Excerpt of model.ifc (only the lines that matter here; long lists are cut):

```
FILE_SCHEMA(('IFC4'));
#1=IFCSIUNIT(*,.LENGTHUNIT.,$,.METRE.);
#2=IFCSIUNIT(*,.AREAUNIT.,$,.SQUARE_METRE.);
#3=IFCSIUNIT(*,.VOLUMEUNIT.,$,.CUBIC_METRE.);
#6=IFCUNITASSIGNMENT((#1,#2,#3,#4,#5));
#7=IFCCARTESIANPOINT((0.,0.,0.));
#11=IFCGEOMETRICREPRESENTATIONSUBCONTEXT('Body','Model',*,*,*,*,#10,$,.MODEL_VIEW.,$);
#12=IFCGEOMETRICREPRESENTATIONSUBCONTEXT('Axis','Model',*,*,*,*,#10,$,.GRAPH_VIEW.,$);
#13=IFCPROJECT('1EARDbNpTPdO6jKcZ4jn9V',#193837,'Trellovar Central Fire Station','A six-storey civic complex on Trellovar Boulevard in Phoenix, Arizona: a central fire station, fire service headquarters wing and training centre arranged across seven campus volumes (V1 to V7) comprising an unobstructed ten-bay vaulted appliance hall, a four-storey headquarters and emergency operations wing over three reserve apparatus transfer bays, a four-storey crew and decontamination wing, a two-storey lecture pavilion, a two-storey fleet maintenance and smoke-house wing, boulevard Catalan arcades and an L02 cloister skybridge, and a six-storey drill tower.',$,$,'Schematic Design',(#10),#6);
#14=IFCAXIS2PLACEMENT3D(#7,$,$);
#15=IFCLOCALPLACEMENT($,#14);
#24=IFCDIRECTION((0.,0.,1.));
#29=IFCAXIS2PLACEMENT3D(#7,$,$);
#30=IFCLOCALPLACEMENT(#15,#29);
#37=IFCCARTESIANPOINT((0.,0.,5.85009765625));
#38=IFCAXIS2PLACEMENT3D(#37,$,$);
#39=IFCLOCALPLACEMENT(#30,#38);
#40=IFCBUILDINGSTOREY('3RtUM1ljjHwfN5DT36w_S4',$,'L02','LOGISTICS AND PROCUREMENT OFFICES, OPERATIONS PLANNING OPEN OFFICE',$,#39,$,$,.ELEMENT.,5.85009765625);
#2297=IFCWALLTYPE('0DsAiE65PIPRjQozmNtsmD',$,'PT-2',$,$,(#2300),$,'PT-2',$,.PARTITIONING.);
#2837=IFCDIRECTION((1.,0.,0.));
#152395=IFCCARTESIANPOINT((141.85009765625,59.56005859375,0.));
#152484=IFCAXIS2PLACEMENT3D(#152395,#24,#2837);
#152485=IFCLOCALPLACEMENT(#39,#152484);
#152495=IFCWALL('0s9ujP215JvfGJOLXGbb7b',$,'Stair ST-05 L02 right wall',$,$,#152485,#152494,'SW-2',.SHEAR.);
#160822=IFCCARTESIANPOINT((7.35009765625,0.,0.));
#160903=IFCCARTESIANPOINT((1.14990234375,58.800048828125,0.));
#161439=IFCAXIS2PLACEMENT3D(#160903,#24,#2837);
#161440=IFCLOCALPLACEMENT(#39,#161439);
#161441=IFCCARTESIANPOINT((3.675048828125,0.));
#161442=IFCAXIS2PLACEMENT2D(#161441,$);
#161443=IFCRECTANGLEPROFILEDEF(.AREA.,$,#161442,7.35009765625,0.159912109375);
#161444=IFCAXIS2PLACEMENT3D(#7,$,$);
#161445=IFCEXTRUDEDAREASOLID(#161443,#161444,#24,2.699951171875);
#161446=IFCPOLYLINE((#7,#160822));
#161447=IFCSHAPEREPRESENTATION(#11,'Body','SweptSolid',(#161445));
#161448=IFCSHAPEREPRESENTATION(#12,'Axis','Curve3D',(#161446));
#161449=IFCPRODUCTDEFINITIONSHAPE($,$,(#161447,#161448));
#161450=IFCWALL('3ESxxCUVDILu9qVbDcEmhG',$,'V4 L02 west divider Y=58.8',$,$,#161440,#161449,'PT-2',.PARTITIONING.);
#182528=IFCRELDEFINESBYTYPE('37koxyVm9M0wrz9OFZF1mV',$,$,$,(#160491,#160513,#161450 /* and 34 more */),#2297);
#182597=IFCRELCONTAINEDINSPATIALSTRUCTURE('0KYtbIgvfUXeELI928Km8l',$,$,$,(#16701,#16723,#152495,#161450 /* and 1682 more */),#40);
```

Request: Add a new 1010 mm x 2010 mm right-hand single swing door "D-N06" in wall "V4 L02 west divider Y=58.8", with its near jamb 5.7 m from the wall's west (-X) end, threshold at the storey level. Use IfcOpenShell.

```python
import numpy as np
import ifcopenshell
import ifcopenshell.api.feature
import ifcopenshell.api.geometry
import ifcopenshell.api.root
import ifcopenshell.api.spatial
import ifcopenshell.geom
import ifcopenshell.util.element
import ifcopenshell.util.placement
import ifcopenshell.util.representation
import ifcopenshell.util.shape
import ifcopenshell.util.unit

model = ifcopenshell.open("model.ifc")
unit_scale = ifcopenshell.util.unit.calculate_unit_scale(model)
settings = ifcopenshell.geom.settings()


def volume(element):
    """Net volume in cubic metres, openings subtracted."""
    shape = ifcopenshell.geom.create_shape(settings, element)
    return ifcopenshell.util.shape.get_volume(shape.geometry)


wall = model.by_id(161450)
storey = ifcopenshell.util.element.get_container(wall, ifc_class="IfcBuildingStorey")
context = ifcopenshell.util.representation.get_context(model, "Model", "Body", "MODEL_VIEW")
before = volume(wall)

width, height, from_end, sill = 1.01, 2.01, 5.7, 0.0  # metres

# The wall runs along its own X axis, and the end named is its -X end.
wall_shape = ifcopenshell.geom.create_shape(settings, wall)
x, y, z = ifcopenshell.util.shape.get_vertices(wall_shape.geometry).T
start = x.min() + from_end
face, thickness = float(y.min()), float(y.max() - y.min())
wall_matrix = ifcopenshell.util.placement.get_local_placement(wall.ObjectPlacement)
level = ifcopenshell.util.placement.get_local_placement(storey.ObjectPlacement)[2, 3]


def in_wall(x, y):
    """Placement at x, y metres in the wall's axes, at sill height."""
    matrix = wall_matrix.copy()
    matrix[:, 3] = wall_matrix @ np.array([x / unit_scale, y / unit_scale, 0.0, 1.0])
    matrix[2, 3] = level + sill / unit_scale
    return matrix


# Opening: a box that overshoots both wall faces by 50 mm.
opening = ifcopenshell.api.root.create_entity(model, ifc_class="IfcOpeningElement", predefined_type="OPENING")
box = ifcopenshell.api.geometry.add_wall_representation(
    model, context=context, length=width, height=height, thickness=thickness + 0.1
)
ifcopenshell.api.geometry.assign_representation(model, product=opening, representation=box)
ifcopenshell.api.geometry.edit_object_placement(model, product=opening, matrix=in_wall(start, face - 0.05), is_si=False)
ifcopenshell.api.feature.add_feature(model, feature=opening, element=wall)

door = ifcopenshell.api.root.create_entity(model, ifc_class="IfcDoor", name="D-N06", predefined_type="DOOR")
door.OverallWidth, door.OverallHeight = width / unit_scale, height / unit_scale
door.OperationType = "SINGLE_SWING_RIGHT"
body = ifcopenshell.api.geometry.add_door_representation(
    model,
    context=context,
    overall_width=door.OverallWidth,
    overall_height=door.OverallHeight,
    operation_type="SINGLE_SWING_RIGHT",
    lining_properties={"LiningDepth": thickness / unit_scale, "ThresholdDepth": thickness / unit_scale},
)
ifcopenshell.api.geometry.assign_representation(model, product=door, representation=body)
ifcopenshell.api.spatial.assign_container(model, products=[door], relating_structure=storey)
ifcopenshell.api.feature.add_filling(model, opening=opening, element=door)

# The lining spans the wall, so the door starts at the wall face.
ifcopenshell.api.geometry.edit_object_placement(model, product=door, matrix=in_wall(start, face), is_si=False)

after = volume(wall)

print(f"wall volume {before:.3f} -> {after:.3f} m3")

model.write("model_updated.ifc")
```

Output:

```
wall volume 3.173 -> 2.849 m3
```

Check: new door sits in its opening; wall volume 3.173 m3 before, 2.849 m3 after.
